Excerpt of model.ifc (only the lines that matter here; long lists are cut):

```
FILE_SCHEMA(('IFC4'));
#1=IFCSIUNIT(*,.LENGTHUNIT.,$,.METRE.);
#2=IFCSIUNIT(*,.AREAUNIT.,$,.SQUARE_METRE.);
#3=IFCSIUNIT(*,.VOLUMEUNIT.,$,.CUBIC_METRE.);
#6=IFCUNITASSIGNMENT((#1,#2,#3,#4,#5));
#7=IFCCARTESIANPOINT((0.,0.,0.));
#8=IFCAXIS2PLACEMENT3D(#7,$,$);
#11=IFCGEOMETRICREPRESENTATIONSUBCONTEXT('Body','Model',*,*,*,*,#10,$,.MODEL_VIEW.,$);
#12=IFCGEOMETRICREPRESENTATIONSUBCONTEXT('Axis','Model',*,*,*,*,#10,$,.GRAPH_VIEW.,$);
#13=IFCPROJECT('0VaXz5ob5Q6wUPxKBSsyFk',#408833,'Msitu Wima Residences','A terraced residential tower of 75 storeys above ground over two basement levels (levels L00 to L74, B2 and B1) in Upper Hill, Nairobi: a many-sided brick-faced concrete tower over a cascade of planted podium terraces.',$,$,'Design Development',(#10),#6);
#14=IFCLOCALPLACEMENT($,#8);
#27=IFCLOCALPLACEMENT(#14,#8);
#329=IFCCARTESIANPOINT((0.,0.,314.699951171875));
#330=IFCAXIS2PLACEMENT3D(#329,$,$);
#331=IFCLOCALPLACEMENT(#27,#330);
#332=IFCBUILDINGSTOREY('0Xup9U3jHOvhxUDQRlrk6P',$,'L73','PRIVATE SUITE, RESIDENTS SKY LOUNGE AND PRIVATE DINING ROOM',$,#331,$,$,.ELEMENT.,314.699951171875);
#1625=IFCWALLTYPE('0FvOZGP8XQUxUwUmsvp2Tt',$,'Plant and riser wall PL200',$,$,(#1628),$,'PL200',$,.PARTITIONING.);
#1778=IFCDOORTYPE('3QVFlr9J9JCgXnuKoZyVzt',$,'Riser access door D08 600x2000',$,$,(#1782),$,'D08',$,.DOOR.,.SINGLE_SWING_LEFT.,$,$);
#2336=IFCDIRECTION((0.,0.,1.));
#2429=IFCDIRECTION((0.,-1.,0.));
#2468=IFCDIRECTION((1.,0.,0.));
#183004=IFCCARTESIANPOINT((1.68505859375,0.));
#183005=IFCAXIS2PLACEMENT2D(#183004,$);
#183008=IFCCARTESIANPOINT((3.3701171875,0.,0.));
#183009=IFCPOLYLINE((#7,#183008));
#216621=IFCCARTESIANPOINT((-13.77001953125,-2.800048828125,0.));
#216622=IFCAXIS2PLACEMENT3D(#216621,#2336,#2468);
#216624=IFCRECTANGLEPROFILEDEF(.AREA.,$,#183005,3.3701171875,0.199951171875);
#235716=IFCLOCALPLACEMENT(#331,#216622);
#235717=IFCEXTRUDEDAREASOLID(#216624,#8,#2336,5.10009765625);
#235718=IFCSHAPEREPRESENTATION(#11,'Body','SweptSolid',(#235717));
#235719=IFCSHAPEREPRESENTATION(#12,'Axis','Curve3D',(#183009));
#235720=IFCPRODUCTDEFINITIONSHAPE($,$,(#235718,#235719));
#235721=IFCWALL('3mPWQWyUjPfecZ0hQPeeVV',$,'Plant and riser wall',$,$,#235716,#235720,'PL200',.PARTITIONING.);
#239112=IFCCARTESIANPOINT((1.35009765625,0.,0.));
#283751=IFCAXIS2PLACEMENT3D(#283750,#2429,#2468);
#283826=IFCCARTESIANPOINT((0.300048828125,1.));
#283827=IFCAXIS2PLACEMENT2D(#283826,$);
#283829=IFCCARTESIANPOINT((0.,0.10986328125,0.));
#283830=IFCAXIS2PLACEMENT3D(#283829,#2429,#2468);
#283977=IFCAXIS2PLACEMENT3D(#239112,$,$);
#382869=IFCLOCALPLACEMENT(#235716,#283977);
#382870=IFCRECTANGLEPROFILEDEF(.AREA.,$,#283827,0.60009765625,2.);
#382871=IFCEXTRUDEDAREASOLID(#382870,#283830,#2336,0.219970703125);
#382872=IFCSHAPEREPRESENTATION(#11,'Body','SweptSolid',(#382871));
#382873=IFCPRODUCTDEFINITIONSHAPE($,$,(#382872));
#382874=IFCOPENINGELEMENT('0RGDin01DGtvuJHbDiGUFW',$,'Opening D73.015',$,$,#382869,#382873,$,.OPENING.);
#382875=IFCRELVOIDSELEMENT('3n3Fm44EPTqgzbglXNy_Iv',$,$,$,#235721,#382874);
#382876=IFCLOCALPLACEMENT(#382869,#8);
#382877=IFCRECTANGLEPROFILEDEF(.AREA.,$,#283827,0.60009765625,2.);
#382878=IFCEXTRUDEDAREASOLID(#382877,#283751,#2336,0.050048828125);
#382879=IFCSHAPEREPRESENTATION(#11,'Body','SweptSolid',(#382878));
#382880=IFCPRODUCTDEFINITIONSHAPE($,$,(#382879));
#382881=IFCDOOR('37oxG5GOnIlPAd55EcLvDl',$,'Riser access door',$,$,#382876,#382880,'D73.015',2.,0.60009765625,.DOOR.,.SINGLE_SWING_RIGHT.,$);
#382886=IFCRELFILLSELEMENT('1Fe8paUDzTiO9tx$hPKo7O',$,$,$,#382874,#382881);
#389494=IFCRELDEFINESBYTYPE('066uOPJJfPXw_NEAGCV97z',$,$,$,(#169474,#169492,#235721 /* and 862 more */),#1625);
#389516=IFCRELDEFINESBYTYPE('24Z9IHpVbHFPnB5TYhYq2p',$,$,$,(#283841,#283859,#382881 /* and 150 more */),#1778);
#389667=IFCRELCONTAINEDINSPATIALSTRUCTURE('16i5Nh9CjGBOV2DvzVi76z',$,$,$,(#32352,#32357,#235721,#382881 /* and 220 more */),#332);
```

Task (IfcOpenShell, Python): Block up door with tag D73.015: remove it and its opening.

```python
import ifcopenshell
import ifcopenshell.api.feature
import ifcopenshell.api.root
import ifcopenshell.geom
import ifcopenshell.util.shape

model = ifcopenshell.open("model.ifc")
settings = ifcopenshell.geom.settings()


def volume(element):
    """Net volume in cubic metres, openings subtracted."""
    shape = ifcopenshell.geom.create_shape(settings, element)
    return ifcopenshell.util.shape.get_volume(shape.geometry)


door = model.by_guid("37oxG5GOnIlPAd55EcLvDl")
opening = door.FillsVoids[0].RelatingOpeningElement
wall = opening.VoidsElements[0].RelatingBuildingElement
before = volume(wall)

ifcopenshell.api.root.remove_product(model, product=door)
ifcopenshell.api.feature.remove_feature(model, feature=opening)

after = volume(wall)

print(f"wall volume {before:.3f} -> {after:.3f} m3")

model.write("model_edited.ifc")
```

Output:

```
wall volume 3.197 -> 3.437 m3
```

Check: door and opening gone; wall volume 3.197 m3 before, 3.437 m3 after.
